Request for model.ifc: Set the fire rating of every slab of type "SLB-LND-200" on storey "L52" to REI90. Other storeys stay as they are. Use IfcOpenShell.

First a look at what the model holds.

```python
import ifcopenshell
import ifcopenshell.util.element

model = ifcopenshell.open("model.ifc")
print(model.schema)
storey = next(s for s in model.by_type("IfcBuildingStorey") if s.Name == "L52")
slabs = [e for e in ifcopenshell.util.element.get_decomposition(storey) if e.is_a("IfcSlab")]
seen = {}
for e in slabs:
    element_type = ifcopenshell.util.element.get_type(e)
    key = (element_type.Name if element_type != e and element_type else None, ifcopenshell.util.element.get_pset(e, "Pset_SlabCommon", "FireRating"))
    seen[key] = seen.get(key, 0) + 1
for (name, value), count in sorted(seen.items(), key=str):
    print(count, "x", name, "|", value)
```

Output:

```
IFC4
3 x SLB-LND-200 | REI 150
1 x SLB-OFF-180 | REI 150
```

```python
import ifcopenshell
import ifcopenshell.api.pset
import ifcopenshell.util.element

model = ifcopenshell.open("model.ifc")

storey = next(s for s in model.by_type("IfcBuildingStorey") if s.Name == "L52")
slabs = [e for e in ifcopenshell.util.element.get_decomposition(storey) if e.is_a("IfcSlab")]

count = 0
for e in slabs:
    element_type = ifcopenshell.util.element.get_type(e)
    if element_type in (None, e) or element_type.Name != "SLB-LND-200":
        continue
    found = ifcopenshell.util.element.get_pset(e, "Pset_SlabCommon", should_inherit=False)
    if found:
        pset = model.by_id(found["id"])
        if len(ifcopenshell.util.element.get_elements_by_pset(pset)) > 1:
            pset = ifcopenshell.api.pset.unshare_pset(model, products=[e], pset=pset)[0]
    else:
        pset = ifcopenshell.api.pset.add_pset(model, product=e, name="Pset_SlabCommon")
    ifcopenshell.api.pset.edit_pset(model, pset=pset, properties={"FireRating": "REI90"})
    count += 1

print(count, "slabs updated")

model.write("model_edited.ifc")
```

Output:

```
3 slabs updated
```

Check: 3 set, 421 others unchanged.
